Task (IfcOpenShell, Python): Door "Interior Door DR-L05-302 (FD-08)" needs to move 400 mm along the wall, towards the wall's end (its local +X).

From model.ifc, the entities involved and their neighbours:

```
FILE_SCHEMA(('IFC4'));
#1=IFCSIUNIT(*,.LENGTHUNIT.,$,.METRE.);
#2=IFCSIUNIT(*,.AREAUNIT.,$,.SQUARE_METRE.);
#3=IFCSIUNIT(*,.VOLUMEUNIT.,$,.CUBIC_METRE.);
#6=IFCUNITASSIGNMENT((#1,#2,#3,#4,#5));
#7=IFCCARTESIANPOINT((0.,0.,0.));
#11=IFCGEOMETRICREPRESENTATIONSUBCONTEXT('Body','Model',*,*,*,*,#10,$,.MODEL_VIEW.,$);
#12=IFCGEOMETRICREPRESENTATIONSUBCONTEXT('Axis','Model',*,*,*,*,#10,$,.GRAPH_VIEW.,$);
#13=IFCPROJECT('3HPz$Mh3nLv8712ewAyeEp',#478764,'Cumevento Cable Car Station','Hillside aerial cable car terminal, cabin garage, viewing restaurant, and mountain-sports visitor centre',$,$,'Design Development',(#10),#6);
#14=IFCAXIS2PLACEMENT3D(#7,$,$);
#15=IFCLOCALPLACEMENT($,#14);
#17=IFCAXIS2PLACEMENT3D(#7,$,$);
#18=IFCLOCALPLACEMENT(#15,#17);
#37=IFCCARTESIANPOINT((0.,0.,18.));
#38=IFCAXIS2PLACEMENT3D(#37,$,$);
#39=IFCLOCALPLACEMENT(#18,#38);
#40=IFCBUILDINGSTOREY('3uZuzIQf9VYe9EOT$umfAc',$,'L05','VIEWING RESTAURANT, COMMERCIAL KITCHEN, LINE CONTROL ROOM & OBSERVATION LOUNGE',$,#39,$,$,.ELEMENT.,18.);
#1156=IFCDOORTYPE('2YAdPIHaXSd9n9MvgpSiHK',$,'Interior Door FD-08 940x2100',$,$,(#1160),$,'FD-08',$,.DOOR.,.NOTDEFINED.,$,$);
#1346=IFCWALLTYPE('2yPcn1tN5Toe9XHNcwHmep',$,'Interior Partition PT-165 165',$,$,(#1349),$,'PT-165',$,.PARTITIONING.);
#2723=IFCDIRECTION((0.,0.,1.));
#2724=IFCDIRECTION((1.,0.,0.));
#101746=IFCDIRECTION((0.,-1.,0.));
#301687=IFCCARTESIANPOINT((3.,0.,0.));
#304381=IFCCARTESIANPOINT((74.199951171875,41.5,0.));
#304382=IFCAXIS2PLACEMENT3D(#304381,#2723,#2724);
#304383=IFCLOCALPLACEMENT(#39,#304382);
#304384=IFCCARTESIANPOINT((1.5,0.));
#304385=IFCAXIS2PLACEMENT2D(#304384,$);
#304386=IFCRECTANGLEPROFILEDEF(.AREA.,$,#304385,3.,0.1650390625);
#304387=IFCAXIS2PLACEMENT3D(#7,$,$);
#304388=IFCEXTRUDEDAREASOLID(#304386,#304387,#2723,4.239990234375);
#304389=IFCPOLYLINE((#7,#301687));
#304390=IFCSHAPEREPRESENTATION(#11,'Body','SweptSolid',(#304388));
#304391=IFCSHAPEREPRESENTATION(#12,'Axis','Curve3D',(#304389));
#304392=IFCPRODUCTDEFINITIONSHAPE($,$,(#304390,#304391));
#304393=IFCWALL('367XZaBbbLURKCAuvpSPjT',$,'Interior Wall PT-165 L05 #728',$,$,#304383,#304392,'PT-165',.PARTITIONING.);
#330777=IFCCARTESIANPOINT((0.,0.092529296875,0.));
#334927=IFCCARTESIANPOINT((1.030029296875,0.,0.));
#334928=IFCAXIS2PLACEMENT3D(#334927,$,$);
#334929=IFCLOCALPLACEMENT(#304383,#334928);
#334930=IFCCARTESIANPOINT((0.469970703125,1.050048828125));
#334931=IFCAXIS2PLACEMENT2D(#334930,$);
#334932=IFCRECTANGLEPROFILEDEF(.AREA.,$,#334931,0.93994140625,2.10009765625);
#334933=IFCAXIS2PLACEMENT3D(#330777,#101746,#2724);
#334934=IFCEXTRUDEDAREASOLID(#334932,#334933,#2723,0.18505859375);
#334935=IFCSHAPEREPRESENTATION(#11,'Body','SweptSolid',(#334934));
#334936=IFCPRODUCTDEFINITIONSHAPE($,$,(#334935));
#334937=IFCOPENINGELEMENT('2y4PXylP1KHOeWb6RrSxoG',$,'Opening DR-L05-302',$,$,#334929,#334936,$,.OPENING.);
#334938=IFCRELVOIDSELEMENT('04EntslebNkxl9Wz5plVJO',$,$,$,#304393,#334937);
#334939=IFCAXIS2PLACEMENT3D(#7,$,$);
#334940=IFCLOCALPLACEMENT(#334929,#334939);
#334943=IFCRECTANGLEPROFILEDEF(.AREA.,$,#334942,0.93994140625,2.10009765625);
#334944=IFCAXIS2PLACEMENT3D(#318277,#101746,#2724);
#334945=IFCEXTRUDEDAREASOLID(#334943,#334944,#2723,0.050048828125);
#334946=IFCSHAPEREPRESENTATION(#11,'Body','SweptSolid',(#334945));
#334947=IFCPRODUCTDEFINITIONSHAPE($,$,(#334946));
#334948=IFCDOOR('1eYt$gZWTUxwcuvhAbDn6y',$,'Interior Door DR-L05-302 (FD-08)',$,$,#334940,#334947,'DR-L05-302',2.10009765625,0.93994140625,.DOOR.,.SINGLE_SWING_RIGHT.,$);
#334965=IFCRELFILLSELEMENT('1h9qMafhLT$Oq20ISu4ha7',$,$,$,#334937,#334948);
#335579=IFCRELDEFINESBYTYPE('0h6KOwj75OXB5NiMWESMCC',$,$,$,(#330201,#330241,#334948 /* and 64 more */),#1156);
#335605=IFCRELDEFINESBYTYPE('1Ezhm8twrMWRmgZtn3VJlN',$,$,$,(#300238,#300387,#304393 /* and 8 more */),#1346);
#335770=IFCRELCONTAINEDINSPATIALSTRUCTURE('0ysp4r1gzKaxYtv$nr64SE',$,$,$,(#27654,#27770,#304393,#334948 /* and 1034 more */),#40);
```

```python
import ifcopenshell
import ifcopenshell.api.geometry
import ifcopenshell.util.placement
import ifcopenshell.util.unit

model = ifcopenshell.open("model.ifc")
unit_scale = ifcopenshell.util.unit.calculate_unit_scale(model)

door = model.by_guid("1eYt$gZWTUxwcuvhAbDn6y")
opening = door.FillsVoids[0].RelatingOpeningElement
wall = opening.VoidsElements[0].RelatingBuildingElement

wall_matrix = ifcopenshell.util.placement.get_local_placement(wall.ObjectPlacement)
shift = wall_matrix[:3, 0] * 0.4 / unit_scale
before = ifcopenshell.util.placement.get_local_placement(door.ObjectPlacement)[:3, 3].copy()

# The door is placed relative to its opening, so it follows when the opening moves.
matrix = ifcopenshell.util.placement.get_local_placement(opening.ObjectPlacement)
matrix[:3, 3] += shift
ifcopenshell.api.geometry.edit_object_placement(
    model, product=opening, matrix=matrix, is_si=False, should_transform_children=True
)

after = ifcopenshell.util.placement.get_local_placement(door.ObjectPlacement)[:3, 3]
print("door moved by", (after - before).round(3) + 0.0)

model.write("model_edited.ifc")
```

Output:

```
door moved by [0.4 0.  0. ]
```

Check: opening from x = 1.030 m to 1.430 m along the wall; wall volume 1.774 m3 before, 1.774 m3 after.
